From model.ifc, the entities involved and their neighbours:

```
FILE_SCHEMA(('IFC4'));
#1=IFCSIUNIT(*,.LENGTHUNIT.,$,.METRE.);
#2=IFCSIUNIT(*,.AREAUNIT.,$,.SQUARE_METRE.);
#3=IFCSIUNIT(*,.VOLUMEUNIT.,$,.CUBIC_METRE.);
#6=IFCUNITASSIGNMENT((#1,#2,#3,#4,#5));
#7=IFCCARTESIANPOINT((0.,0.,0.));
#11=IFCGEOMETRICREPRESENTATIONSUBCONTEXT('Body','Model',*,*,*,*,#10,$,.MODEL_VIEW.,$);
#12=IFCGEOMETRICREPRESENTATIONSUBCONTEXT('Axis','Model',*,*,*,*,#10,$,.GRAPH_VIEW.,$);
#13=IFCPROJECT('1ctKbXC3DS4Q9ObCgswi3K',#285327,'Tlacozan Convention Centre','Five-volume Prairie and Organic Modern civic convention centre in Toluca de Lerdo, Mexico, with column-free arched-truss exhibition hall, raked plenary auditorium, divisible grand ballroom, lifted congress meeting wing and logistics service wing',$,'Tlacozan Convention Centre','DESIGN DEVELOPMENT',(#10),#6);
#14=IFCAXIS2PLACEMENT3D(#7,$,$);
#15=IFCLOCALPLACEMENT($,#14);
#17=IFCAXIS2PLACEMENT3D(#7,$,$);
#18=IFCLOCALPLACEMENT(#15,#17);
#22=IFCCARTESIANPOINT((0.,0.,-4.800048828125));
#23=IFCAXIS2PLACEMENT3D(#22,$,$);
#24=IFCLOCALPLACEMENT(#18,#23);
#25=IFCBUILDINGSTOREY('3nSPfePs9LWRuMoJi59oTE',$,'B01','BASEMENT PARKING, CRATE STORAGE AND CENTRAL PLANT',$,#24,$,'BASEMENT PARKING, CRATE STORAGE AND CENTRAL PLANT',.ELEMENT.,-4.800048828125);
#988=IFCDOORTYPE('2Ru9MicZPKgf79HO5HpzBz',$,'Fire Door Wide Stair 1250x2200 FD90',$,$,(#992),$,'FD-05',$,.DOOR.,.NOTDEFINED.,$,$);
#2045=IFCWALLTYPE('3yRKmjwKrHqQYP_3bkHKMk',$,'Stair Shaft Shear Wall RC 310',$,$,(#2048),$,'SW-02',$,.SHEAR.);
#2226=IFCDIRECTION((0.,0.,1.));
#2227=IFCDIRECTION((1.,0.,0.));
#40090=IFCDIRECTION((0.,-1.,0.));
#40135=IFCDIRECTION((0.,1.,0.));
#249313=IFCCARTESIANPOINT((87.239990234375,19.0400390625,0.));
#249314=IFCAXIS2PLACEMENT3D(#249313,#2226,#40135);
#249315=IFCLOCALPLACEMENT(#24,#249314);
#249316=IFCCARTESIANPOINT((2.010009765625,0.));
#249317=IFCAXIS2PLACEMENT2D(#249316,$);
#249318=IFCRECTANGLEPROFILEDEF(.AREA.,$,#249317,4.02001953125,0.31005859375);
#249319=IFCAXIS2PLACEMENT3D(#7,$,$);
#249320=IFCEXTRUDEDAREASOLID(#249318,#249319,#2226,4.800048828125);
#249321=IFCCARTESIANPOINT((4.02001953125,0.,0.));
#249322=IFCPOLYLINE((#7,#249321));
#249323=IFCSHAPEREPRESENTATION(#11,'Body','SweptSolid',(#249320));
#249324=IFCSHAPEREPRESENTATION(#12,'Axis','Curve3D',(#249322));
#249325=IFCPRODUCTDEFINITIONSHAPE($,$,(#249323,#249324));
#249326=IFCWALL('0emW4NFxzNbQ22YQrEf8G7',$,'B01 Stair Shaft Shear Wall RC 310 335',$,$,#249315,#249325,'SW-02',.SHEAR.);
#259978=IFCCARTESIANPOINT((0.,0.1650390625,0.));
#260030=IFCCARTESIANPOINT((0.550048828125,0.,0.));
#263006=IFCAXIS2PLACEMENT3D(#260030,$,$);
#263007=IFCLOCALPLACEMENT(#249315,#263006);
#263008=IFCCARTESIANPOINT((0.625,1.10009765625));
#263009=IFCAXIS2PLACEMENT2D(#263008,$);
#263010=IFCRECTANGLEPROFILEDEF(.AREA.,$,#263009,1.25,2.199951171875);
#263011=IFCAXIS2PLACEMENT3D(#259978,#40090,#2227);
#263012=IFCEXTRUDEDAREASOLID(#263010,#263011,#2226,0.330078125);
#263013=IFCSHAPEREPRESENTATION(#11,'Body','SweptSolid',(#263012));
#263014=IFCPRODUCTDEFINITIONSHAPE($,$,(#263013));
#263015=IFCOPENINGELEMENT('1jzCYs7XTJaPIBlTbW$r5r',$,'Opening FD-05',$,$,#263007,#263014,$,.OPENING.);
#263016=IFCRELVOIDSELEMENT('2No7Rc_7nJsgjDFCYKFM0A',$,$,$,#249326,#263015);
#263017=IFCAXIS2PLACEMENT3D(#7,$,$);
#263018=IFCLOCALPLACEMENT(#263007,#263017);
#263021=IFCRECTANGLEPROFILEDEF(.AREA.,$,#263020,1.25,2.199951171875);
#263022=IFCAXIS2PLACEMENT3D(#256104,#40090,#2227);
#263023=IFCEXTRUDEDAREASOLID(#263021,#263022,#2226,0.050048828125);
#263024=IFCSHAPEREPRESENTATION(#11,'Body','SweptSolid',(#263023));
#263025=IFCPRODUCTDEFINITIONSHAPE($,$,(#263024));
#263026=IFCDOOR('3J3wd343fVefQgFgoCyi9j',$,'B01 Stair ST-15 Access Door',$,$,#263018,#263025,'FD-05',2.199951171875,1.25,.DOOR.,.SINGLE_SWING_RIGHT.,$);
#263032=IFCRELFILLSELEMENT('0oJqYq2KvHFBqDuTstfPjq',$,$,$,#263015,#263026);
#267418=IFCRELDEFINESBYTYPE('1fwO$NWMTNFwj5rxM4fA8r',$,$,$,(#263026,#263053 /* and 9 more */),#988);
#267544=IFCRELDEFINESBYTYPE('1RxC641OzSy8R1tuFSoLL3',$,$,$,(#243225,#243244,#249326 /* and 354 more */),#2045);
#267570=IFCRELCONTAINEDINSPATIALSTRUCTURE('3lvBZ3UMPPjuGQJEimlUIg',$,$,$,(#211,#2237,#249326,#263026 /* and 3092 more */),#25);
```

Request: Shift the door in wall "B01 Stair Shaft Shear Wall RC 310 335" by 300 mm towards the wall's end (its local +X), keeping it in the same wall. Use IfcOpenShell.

```python
import ifcopenshell
import ifcopenshell.api.geometry
import ifcopenshell.util.placement

model = ifcopenshell.open("model.ifc")

door = model.by_id(263026)
opening = door.FillsVoids[0].RelatingOpeningElement
wall = opening.VoidsElements[0].RelatingBuildingElement

wall_matrix = ifcopenshell.util.placement.get_local_placement(wall.ObjectPlacement)
shift = wall_matrix[:3, 0] * 0.3
before = ifcopenshell.util.placement.get_local_placement(door.ObjectPlacement)[:3, 3].copy()

# The door is placed relative to its opening, so it follows when the opening moves.
matrix = ifcopenshell.util.placement.get_local_placement(opening.ObjectPlacement)
matrix[:3, 3] += shift
ifcopenshell.api.geometry.edit_object_placement(
    model, product=opening, matrix=matrix, is_si=False, should_transform_children=True
)

after = ifcopenshell.util.placement.get_local_placement(door.ObjectPlacement)[:3, 3]
print("door moved by", (after - before).round(3) + 0.0)

model.write("model_rev.ifc")
```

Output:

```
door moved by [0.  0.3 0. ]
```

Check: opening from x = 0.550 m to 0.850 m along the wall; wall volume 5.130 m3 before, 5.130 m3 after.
